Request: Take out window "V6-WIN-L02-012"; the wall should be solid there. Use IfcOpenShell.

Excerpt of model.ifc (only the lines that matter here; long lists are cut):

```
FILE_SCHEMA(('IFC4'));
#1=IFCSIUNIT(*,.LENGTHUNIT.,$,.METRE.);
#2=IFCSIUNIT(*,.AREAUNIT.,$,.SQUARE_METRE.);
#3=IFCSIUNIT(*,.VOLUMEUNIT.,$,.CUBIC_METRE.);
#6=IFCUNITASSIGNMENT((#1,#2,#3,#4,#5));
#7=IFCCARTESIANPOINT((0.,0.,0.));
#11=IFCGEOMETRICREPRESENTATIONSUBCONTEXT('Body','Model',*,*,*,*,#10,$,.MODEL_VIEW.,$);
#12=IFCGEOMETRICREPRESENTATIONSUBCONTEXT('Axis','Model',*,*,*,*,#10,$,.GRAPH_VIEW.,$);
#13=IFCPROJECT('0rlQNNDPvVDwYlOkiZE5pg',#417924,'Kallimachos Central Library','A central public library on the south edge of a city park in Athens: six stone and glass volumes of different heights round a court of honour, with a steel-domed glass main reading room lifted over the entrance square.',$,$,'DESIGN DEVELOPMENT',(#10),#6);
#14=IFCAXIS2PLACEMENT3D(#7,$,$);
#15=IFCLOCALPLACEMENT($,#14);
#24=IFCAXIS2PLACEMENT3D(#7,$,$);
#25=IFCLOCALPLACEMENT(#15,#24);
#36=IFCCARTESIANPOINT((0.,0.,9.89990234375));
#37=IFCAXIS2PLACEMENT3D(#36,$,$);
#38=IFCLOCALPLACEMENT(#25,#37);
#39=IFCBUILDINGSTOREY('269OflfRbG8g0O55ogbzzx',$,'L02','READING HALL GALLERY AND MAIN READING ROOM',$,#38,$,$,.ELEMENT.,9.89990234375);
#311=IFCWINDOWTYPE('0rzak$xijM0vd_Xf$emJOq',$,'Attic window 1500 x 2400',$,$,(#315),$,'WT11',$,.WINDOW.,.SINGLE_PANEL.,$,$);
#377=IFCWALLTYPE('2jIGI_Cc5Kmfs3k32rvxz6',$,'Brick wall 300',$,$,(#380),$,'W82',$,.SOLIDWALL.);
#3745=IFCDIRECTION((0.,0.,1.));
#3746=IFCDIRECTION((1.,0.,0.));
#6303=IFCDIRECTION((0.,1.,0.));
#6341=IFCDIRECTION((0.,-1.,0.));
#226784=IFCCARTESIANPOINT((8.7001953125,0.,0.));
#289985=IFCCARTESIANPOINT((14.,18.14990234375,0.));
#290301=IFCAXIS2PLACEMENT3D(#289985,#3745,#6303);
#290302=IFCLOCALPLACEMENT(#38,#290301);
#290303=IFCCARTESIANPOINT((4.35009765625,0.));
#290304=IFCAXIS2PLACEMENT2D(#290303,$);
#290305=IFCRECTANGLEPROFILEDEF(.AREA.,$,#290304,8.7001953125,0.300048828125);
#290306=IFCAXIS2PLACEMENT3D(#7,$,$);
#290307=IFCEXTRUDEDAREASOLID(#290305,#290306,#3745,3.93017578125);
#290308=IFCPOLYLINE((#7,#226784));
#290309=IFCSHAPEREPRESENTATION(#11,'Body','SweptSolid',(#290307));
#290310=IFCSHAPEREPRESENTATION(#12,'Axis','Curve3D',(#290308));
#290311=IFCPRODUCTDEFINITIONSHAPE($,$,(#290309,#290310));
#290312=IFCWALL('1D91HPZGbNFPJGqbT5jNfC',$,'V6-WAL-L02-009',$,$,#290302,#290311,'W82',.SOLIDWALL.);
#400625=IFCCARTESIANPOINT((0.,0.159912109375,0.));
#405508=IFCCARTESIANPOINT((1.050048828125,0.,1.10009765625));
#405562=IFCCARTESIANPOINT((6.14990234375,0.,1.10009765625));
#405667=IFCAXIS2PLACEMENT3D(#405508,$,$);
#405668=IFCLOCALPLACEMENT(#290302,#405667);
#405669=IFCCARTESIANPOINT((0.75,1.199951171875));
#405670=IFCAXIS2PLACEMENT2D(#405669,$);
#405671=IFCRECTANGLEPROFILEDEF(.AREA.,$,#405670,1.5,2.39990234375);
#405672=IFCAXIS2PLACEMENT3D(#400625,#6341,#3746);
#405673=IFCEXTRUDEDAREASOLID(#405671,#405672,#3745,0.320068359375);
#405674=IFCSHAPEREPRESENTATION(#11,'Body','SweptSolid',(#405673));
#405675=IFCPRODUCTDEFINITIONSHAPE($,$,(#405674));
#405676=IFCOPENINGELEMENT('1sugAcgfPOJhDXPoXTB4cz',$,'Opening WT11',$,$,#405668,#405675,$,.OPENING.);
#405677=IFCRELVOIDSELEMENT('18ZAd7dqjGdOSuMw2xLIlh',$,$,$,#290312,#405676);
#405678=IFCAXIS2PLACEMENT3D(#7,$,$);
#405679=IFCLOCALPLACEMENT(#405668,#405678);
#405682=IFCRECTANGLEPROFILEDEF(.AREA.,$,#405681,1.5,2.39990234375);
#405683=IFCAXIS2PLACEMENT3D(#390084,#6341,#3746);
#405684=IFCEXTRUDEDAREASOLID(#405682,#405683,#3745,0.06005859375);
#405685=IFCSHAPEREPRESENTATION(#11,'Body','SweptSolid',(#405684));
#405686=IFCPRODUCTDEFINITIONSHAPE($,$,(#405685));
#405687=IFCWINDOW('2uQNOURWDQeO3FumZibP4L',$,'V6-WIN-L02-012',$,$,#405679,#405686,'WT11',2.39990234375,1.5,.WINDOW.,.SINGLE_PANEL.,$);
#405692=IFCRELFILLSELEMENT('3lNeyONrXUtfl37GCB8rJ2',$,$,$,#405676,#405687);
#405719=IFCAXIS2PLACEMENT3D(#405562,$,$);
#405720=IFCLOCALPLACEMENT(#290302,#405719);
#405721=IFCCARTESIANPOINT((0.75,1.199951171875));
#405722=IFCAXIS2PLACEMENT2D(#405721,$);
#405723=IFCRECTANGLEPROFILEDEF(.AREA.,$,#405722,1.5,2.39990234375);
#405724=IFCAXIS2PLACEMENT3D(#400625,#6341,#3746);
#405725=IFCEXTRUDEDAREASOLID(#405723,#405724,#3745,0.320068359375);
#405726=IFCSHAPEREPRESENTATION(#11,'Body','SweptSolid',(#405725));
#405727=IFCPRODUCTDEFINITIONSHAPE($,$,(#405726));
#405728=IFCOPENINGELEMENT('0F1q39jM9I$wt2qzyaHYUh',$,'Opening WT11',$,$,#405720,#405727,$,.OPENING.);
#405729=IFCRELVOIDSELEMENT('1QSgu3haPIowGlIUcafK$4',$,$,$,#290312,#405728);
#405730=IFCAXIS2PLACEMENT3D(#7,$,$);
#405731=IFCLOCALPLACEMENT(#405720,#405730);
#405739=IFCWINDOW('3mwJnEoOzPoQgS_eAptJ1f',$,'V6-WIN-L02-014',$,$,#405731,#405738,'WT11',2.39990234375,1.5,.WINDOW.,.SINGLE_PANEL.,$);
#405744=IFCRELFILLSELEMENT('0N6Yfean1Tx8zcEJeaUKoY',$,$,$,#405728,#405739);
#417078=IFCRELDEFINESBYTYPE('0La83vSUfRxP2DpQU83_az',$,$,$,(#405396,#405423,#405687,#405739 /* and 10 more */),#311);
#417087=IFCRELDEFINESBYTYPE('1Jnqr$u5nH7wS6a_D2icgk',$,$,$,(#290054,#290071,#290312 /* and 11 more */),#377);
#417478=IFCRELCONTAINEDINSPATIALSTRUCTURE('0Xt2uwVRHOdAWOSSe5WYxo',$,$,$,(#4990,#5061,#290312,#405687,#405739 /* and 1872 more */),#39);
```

```python
import ifcopenshell
import ifcopenshell.api.feature
import ifcopenshell.api.root
import ifcopenshell.geom
import ifcopenshell.util.shape

model = ifcopenshell.open("model.ifc")
settings = ifcopenshell.geom.settings()


def volume(element):
    """Net volume in cubic metres, openings subtracted."""
    shape = ifcopenshell.geom.create_shape(settings, element)
    return ifcopenshell.util.shape.get_volume(shape.geometry)


window = model.by_guid("2uQNOURWDQeO3FumZibP4L")
opening = window.FillsVoids[0].RelatingOpeningElement
wall = opening.VoidsElements[0].RelatingBuildingElement
before = volume(wall)

ifcopenshell.api.root.remove_product(model, product=window)
ifcopenshell.api.feature.remove_feature(model, feature=opening)

after = volume(wall)

print(f"wall volume {before:.3f} -> {after:.3f} m3")

model.write("model_edited.ifc")
```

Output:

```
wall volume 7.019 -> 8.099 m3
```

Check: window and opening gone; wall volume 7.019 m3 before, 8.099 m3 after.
